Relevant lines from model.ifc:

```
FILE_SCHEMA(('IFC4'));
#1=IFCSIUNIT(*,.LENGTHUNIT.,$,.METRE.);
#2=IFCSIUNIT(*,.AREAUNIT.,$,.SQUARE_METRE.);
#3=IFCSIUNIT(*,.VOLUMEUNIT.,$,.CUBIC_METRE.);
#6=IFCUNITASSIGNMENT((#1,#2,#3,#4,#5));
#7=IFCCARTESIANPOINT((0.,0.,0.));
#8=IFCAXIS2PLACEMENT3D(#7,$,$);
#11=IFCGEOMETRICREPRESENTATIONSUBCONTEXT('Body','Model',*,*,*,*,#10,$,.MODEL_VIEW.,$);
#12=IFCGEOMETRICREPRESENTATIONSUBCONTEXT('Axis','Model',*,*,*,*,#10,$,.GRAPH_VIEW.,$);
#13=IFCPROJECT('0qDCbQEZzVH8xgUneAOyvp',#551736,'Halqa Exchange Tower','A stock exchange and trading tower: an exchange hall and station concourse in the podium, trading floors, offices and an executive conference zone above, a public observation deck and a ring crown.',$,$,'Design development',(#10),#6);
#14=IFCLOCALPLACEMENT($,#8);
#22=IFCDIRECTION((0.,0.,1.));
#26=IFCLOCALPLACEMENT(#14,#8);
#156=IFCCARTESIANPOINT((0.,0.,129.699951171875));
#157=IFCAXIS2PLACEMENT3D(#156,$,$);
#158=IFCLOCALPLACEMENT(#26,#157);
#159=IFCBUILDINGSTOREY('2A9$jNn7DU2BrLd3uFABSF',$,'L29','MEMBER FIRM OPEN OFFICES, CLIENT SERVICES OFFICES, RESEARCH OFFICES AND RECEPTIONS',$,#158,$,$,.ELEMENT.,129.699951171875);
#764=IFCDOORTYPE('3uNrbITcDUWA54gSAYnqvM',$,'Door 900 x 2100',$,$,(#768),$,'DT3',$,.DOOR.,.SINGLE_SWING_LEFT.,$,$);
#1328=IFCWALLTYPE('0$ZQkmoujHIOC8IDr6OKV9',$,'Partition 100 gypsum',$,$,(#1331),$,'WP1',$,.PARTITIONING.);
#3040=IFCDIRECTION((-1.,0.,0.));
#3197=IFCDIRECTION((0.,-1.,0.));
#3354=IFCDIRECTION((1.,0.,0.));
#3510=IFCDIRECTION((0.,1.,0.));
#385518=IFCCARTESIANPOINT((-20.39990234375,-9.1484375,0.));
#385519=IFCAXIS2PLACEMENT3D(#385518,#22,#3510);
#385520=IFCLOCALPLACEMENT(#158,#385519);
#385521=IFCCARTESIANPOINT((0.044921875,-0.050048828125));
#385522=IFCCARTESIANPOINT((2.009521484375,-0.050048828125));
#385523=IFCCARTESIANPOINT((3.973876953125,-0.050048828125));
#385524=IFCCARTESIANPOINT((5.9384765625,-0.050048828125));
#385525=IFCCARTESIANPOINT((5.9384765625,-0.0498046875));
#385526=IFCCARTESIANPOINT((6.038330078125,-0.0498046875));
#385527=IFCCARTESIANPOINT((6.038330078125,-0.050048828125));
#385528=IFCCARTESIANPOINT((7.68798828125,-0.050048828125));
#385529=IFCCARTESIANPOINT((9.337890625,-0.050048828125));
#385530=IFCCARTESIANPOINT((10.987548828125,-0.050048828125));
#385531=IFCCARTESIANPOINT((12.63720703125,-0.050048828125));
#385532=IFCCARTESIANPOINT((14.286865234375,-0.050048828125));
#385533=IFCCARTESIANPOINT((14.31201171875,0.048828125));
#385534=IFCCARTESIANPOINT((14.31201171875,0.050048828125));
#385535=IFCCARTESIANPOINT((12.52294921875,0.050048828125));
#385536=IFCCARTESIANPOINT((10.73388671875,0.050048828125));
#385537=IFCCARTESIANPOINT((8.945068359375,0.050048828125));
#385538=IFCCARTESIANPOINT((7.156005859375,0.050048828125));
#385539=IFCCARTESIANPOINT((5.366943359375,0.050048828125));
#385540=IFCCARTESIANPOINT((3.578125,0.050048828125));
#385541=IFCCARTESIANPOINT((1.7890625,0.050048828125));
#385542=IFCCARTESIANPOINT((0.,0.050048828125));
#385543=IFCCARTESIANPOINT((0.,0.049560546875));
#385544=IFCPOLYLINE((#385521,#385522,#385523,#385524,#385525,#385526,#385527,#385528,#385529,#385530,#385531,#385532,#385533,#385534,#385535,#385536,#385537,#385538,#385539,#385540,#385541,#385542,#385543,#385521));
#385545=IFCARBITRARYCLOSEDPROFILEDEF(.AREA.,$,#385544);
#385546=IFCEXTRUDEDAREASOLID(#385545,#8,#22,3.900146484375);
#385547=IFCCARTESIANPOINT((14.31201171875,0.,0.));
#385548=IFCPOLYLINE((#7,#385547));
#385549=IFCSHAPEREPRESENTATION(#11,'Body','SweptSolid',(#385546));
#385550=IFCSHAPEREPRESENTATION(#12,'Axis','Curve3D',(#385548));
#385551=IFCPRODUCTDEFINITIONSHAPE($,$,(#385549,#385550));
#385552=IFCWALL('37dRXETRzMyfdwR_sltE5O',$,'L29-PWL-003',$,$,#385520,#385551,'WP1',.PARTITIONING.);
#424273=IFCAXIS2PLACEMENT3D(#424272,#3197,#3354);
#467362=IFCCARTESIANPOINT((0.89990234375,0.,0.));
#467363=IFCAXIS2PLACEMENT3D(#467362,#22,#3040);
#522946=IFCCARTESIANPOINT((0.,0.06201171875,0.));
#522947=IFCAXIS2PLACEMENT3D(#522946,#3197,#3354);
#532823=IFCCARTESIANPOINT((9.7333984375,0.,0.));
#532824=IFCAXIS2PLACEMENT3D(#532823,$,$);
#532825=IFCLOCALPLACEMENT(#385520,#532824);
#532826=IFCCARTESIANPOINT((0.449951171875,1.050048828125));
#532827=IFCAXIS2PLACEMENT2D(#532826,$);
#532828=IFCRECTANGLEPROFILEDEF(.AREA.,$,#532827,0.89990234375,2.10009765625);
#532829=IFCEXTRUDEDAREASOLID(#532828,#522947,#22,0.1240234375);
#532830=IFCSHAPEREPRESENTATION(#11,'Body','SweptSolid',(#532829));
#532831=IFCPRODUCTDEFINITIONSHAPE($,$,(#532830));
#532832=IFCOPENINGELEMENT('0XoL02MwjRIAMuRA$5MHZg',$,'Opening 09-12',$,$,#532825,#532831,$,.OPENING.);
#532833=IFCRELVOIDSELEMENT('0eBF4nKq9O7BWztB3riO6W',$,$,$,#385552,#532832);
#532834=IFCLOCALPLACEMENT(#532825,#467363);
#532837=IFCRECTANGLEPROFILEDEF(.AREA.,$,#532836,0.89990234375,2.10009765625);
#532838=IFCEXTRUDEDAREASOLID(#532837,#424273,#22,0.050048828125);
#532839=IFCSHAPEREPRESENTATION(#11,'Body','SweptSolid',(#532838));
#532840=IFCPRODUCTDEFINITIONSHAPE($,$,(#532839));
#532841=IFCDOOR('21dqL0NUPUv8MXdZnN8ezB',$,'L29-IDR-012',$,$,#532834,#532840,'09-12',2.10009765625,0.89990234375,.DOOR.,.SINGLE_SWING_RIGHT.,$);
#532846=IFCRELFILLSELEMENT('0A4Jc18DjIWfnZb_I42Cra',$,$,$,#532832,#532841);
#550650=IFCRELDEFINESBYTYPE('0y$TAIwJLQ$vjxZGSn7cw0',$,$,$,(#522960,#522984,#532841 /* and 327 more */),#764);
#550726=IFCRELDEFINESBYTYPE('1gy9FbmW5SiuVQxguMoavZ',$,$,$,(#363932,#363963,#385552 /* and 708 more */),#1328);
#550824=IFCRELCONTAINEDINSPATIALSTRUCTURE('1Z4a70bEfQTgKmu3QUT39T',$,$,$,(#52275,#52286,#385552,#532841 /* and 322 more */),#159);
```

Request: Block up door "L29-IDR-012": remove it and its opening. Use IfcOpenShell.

```python
import ifcopenshell
import ifcopenshell.api.feature
import ifcopenshell.api.root
import ifcopenshell.geom
import ifcopenshell.util.shape

model = ifcopenshell.open("model.ifc")
settings = ifcopenshell.geom.settings()


def volume(element):
    """Net volume in cubic metres, openings subtracted."""
    shape = ifcopenshell.geom.create_shape(settings, element)
    return ifcopenshell.util.shape.get_volume(shape.geometry)


door = model.by_guid("21dqL0NUPUv8MXdZnN8ezB")
opening = door.FillsVoids[0].RelatingOpeningElement
wall = opening.VoidsElements[0].RelatingBuildingElement
before = volume(wall)

ifcopenshell.api.root.remove_product(model, product=door)
ifcopenshell.api.feature.remove_feature(model, feature=opening)

after = volume(wall)

print(f"wall volume {before:.3f} -> {after:.3f} m3")

model.write("model-out.ifc")
```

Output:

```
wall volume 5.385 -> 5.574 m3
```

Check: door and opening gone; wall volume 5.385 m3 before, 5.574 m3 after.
